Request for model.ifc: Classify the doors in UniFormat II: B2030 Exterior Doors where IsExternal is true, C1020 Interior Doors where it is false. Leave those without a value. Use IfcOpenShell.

First a look at what the model holds.

```python
import ifcopenshell
import ifcopenshell.util.element

model = ifcopenshell.open("model.ifc")
print(model.schema)
print("classifications:", [c.Name for c in model.by_type("IfcClassification")])
values = [ifcopenshell.util.element.get_pset(e, "Pset_DoorCommon", "IsExternal") for e in model.by_type("IfcDoor")]
for value in (True, False, None):
    print("IsExternal", value, values.count(value))
```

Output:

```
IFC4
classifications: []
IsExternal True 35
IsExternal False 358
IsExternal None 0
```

```python
import ifcopenshell
import ifcopenshell.api.classification
import ifcopenshell.util.element

model = ifcopenshell.open("model.ifc")

system = ifcopenshell.api.classification.add_classification(model, classification="UniFormat II")

doors = model.by_type("IfcDoor")
external = {e: ifcopenshell.util.element.get_pset(e, "Pset_DoorCommon", "IsExternal") for e in doors}
for flag, code, name in ((True, "B2030", "Exterior Doors"), (False, "C1020", "Interior Doors")):
    products = [e for e in doors if external[e] is flag]
    ifcopenshell.api.classification.add_reference(
        model, products=products, classification=system, identification=code, name=name
    )
    print(code, len(products))

model.write("model_v2.ifc")
```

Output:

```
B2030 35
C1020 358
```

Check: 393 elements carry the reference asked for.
